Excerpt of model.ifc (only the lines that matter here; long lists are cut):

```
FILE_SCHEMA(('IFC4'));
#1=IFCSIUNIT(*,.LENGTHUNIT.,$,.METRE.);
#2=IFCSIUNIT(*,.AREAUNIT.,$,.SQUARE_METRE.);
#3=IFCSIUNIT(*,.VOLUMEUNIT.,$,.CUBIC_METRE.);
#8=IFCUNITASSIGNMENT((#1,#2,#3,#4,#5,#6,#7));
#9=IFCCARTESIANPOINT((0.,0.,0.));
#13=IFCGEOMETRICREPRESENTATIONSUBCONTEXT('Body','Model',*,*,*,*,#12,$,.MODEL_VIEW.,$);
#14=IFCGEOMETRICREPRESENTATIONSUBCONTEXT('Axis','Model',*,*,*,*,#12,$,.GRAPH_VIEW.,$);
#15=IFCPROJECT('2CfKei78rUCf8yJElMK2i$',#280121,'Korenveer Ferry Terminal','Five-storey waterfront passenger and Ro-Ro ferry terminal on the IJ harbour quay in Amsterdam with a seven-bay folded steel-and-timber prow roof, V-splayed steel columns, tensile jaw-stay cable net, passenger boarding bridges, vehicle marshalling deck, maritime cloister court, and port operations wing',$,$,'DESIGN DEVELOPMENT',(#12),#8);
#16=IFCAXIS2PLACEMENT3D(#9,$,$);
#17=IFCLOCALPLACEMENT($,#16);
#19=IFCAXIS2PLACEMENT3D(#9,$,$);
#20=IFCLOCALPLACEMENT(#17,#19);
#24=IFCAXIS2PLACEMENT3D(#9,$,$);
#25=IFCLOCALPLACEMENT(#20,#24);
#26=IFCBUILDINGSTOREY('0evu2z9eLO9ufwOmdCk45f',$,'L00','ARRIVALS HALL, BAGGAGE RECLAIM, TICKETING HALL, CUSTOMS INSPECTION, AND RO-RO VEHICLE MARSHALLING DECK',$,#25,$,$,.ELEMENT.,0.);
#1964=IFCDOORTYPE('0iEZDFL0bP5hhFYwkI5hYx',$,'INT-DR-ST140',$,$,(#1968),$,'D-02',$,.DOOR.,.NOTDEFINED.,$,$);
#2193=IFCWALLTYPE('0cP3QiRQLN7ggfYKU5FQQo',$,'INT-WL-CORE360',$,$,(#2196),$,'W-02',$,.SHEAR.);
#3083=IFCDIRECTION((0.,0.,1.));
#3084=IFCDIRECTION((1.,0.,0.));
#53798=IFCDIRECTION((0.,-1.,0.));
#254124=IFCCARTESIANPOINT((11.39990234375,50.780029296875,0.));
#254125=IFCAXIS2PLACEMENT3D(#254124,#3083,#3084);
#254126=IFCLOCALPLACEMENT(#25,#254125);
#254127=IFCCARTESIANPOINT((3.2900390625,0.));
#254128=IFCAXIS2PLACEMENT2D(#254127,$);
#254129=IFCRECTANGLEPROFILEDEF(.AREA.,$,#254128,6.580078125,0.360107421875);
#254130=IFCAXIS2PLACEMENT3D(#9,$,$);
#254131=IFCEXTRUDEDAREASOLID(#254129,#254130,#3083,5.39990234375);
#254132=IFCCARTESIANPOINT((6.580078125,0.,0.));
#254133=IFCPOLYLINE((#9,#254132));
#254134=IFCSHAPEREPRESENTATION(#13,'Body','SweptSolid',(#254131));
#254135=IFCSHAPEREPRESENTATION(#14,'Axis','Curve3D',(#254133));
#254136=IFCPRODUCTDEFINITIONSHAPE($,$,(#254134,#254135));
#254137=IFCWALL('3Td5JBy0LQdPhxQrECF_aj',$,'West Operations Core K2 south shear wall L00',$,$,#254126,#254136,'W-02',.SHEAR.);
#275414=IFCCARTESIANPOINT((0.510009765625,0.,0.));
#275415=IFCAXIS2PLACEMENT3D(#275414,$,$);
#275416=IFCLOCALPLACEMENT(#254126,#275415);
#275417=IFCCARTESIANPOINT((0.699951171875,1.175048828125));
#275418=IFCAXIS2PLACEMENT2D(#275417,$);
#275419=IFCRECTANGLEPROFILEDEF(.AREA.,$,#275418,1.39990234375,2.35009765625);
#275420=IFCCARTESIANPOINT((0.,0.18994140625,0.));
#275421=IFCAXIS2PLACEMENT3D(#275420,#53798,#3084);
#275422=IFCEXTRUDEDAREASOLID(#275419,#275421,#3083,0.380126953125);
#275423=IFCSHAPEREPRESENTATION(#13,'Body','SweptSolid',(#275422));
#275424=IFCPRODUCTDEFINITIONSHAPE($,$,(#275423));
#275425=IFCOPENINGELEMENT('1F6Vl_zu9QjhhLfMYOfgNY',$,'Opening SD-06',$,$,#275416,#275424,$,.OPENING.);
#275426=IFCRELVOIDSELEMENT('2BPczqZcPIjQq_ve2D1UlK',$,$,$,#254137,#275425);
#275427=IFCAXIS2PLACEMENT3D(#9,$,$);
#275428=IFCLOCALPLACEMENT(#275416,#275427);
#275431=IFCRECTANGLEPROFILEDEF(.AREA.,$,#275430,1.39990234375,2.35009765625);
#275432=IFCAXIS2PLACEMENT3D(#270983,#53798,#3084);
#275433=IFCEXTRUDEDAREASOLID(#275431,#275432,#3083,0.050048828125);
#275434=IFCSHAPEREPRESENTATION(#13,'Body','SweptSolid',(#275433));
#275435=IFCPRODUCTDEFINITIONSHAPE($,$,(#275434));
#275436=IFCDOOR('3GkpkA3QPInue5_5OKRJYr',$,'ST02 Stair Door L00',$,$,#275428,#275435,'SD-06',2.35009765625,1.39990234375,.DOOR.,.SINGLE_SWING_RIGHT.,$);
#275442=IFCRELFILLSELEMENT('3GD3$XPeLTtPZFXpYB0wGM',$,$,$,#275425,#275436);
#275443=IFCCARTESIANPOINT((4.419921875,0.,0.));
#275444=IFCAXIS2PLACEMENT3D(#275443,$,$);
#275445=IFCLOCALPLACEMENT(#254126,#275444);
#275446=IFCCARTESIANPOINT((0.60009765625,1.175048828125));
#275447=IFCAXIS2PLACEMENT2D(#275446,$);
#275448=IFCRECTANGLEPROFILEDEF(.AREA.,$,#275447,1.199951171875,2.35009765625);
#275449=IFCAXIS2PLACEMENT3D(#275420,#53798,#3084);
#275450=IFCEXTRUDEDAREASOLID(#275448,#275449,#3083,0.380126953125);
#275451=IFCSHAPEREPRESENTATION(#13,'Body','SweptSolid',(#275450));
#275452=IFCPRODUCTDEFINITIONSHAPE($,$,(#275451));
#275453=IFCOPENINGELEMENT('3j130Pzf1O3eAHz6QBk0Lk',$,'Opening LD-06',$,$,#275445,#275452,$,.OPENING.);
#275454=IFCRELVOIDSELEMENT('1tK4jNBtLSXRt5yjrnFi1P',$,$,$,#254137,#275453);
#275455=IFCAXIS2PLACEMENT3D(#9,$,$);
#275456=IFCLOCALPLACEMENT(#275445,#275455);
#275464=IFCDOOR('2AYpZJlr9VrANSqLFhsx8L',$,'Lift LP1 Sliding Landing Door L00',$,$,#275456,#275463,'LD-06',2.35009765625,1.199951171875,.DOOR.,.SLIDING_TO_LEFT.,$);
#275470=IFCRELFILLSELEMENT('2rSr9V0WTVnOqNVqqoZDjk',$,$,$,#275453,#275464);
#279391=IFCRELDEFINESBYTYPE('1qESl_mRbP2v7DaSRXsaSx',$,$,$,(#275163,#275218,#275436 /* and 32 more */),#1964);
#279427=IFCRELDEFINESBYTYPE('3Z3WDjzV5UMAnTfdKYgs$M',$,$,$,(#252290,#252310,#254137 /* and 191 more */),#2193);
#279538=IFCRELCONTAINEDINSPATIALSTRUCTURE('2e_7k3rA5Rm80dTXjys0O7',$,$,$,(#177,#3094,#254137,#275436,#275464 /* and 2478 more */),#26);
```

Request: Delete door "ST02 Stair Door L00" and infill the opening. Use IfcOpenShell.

```python
import ifcopenshell
import ifcopenshell.api.feature
import ifcopenshell.api.root
import ifcopenshell.geom
import ifcopenshell.util.shape

model = ifcopenshell.open("model.ifc")
settings = ifcopenshell.geom.settings()


def volume(element):
    """Net volume in cubic metres, openings subtracted."""
    shape = ifcopenshell.geom.create_shape(settings, element)
    return ifcopenshell.util.shape.get_volume(shape.geometry)


door = model.by_guid("3GkpkA3QPInue5_5OKRJYr")
opening = door.FillsVoids[0].RelatingOpeningElement
wall = opening.VoidsElements[0].RelatingBuildingElement
before = volume(wall)

ifcopenshell.api.root.remove_product(model, product=door)
ifcopenshell.api.feature.remove_feature(model, feature=opening)

after = volume(wall)

print(f"wall volume {before:.3f} -> {after:.3f} m3")

model.write("model-out.ifc")
```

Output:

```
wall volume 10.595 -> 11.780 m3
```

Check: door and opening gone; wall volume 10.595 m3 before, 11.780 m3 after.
